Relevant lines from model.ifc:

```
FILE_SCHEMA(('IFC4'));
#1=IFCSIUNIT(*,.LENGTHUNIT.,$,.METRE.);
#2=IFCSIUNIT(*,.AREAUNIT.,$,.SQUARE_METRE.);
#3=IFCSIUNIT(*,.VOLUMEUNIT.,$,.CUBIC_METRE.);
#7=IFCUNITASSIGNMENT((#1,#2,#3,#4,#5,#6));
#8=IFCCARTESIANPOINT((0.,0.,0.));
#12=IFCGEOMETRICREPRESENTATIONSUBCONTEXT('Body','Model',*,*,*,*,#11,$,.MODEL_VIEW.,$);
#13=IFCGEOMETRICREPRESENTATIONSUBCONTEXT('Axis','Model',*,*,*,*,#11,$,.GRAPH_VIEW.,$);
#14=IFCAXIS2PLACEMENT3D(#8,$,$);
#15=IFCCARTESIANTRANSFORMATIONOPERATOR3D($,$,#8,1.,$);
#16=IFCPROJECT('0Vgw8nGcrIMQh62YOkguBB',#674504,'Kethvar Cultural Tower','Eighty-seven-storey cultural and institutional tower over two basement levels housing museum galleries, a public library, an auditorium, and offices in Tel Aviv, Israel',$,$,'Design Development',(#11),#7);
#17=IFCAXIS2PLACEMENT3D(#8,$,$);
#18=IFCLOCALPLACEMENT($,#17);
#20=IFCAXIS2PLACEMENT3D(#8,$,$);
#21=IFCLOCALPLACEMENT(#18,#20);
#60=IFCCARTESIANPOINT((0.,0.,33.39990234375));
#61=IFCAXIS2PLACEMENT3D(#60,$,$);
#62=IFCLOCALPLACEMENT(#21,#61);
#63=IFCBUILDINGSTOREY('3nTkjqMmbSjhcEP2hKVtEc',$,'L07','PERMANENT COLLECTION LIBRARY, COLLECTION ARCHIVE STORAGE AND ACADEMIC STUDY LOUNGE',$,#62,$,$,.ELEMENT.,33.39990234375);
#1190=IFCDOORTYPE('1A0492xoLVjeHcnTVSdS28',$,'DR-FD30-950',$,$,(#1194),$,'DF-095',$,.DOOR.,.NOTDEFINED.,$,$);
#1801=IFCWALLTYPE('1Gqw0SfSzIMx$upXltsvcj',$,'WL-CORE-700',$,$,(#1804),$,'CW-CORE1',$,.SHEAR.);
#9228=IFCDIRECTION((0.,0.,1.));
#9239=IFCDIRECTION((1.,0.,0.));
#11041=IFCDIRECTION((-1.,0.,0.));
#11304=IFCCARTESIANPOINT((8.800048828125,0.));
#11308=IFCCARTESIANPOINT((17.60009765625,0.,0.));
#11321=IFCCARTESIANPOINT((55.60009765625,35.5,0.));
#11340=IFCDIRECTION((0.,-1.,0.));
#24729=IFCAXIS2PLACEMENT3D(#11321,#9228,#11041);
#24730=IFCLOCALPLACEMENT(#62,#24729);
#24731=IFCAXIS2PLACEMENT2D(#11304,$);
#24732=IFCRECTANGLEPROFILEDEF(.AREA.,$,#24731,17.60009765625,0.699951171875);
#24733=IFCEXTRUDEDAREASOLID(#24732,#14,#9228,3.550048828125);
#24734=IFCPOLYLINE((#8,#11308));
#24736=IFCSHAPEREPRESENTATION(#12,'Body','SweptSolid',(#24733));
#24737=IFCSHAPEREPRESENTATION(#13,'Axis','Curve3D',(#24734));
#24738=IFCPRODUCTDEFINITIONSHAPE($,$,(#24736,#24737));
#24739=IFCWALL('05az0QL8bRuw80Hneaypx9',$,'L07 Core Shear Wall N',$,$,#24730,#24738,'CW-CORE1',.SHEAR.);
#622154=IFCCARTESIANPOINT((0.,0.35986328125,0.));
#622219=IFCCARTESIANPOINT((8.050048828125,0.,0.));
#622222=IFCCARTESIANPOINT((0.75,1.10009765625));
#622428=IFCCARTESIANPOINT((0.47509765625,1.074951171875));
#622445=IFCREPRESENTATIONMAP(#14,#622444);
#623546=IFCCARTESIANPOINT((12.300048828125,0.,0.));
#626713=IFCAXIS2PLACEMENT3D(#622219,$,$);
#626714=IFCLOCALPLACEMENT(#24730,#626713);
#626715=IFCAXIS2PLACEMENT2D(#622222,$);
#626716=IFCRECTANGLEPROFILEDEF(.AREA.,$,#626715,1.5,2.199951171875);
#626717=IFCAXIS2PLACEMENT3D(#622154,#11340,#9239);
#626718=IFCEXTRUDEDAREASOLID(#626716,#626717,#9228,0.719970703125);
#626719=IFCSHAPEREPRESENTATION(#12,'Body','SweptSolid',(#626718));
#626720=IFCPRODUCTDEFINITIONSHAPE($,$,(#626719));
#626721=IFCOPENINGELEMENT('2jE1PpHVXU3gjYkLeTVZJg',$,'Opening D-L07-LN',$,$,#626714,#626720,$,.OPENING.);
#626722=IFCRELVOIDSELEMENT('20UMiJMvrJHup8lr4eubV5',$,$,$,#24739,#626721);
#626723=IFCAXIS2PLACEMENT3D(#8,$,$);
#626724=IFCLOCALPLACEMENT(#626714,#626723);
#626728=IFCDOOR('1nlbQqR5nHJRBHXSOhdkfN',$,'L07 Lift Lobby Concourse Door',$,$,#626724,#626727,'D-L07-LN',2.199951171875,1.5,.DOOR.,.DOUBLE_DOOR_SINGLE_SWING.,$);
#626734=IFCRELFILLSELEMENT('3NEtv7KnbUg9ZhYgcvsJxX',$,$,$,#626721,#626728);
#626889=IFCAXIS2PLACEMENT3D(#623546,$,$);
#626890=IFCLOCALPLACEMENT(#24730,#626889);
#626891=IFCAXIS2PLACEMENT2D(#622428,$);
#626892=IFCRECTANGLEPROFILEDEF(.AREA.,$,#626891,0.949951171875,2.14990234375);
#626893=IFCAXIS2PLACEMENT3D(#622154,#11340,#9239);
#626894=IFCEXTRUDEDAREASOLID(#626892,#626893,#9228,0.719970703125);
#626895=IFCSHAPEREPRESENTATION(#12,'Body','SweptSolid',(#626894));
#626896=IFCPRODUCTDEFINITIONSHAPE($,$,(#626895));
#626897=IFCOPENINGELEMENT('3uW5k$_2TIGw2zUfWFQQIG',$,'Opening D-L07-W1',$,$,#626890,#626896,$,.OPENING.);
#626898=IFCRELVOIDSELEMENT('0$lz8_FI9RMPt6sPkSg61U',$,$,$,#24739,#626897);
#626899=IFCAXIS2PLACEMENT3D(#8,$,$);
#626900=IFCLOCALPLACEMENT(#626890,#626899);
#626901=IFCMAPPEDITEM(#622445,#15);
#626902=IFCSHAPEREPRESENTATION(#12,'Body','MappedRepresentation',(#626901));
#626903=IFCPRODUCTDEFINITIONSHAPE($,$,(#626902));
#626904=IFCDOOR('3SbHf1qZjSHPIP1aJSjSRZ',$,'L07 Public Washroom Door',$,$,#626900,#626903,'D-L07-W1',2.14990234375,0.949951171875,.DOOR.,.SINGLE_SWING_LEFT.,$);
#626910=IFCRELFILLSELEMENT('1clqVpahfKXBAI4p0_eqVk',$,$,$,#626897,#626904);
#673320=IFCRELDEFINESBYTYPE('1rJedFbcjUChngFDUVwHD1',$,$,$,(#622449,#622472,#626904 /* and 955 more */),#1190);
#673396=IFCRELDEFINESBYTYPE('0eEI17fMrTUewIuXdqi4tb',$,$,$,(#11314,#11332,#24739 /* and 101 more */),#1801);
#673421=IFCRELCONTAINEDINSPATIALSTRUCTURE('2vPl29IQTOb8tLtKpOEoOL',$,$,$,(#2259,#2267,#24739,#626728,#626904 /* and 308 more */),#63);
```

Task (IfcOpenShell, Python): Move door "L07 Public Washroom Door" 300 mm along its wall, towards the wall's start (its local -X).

```python
import ifcopenshell
import ifcopenshell.api.geometry
import ifcopenshell.util.placement
import ifcopenshell.util.unit

model = ifcopenshell.open("model.ifc")
unit_scale = ifcopenshell.util.unit.calculate_unit_scale(model)

door = model.by_guid("3SbHf1qZjSHPIP1aJSjSRZ")
opening = door.FillsVoids[0].RelatingOpeningElement
wall = opening.VoidsElements[0].RelatingBuildingElement

wall_matrix = ifcopenshell.util.placement.get_local_placement(wall.ObjectPlacement)
shift = wall_matrix[:3, 0] * -0.3 / unit_scale
before = ifcopenshell.util.placement.get_local_placement(door.ObjectPlacement)[:3, 3].copy()

# The door is placed relative to its opening, so it follows when the opening moves.
matrix = ifcopenshell.util.placement.get_local_placement(opening.ObjectPlacement)
matrix[:3, 3] += shift
ifcopenshell.api.geometry.edit_object_placement(
    model, product=opening, matrix=matrix, is_si=False, should_transform_children=True
)

after = ifcopenshell.util.placement.get_local_placement(door.ObjectPlacement)[:3, 3]
print("door moved by", (after - before).round(3) + 0.0)

model.write("model_edited.ifc")
```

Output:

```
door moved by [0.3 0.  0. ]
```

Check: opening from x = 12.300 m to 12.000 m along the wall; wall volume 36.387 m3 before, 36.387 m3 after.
